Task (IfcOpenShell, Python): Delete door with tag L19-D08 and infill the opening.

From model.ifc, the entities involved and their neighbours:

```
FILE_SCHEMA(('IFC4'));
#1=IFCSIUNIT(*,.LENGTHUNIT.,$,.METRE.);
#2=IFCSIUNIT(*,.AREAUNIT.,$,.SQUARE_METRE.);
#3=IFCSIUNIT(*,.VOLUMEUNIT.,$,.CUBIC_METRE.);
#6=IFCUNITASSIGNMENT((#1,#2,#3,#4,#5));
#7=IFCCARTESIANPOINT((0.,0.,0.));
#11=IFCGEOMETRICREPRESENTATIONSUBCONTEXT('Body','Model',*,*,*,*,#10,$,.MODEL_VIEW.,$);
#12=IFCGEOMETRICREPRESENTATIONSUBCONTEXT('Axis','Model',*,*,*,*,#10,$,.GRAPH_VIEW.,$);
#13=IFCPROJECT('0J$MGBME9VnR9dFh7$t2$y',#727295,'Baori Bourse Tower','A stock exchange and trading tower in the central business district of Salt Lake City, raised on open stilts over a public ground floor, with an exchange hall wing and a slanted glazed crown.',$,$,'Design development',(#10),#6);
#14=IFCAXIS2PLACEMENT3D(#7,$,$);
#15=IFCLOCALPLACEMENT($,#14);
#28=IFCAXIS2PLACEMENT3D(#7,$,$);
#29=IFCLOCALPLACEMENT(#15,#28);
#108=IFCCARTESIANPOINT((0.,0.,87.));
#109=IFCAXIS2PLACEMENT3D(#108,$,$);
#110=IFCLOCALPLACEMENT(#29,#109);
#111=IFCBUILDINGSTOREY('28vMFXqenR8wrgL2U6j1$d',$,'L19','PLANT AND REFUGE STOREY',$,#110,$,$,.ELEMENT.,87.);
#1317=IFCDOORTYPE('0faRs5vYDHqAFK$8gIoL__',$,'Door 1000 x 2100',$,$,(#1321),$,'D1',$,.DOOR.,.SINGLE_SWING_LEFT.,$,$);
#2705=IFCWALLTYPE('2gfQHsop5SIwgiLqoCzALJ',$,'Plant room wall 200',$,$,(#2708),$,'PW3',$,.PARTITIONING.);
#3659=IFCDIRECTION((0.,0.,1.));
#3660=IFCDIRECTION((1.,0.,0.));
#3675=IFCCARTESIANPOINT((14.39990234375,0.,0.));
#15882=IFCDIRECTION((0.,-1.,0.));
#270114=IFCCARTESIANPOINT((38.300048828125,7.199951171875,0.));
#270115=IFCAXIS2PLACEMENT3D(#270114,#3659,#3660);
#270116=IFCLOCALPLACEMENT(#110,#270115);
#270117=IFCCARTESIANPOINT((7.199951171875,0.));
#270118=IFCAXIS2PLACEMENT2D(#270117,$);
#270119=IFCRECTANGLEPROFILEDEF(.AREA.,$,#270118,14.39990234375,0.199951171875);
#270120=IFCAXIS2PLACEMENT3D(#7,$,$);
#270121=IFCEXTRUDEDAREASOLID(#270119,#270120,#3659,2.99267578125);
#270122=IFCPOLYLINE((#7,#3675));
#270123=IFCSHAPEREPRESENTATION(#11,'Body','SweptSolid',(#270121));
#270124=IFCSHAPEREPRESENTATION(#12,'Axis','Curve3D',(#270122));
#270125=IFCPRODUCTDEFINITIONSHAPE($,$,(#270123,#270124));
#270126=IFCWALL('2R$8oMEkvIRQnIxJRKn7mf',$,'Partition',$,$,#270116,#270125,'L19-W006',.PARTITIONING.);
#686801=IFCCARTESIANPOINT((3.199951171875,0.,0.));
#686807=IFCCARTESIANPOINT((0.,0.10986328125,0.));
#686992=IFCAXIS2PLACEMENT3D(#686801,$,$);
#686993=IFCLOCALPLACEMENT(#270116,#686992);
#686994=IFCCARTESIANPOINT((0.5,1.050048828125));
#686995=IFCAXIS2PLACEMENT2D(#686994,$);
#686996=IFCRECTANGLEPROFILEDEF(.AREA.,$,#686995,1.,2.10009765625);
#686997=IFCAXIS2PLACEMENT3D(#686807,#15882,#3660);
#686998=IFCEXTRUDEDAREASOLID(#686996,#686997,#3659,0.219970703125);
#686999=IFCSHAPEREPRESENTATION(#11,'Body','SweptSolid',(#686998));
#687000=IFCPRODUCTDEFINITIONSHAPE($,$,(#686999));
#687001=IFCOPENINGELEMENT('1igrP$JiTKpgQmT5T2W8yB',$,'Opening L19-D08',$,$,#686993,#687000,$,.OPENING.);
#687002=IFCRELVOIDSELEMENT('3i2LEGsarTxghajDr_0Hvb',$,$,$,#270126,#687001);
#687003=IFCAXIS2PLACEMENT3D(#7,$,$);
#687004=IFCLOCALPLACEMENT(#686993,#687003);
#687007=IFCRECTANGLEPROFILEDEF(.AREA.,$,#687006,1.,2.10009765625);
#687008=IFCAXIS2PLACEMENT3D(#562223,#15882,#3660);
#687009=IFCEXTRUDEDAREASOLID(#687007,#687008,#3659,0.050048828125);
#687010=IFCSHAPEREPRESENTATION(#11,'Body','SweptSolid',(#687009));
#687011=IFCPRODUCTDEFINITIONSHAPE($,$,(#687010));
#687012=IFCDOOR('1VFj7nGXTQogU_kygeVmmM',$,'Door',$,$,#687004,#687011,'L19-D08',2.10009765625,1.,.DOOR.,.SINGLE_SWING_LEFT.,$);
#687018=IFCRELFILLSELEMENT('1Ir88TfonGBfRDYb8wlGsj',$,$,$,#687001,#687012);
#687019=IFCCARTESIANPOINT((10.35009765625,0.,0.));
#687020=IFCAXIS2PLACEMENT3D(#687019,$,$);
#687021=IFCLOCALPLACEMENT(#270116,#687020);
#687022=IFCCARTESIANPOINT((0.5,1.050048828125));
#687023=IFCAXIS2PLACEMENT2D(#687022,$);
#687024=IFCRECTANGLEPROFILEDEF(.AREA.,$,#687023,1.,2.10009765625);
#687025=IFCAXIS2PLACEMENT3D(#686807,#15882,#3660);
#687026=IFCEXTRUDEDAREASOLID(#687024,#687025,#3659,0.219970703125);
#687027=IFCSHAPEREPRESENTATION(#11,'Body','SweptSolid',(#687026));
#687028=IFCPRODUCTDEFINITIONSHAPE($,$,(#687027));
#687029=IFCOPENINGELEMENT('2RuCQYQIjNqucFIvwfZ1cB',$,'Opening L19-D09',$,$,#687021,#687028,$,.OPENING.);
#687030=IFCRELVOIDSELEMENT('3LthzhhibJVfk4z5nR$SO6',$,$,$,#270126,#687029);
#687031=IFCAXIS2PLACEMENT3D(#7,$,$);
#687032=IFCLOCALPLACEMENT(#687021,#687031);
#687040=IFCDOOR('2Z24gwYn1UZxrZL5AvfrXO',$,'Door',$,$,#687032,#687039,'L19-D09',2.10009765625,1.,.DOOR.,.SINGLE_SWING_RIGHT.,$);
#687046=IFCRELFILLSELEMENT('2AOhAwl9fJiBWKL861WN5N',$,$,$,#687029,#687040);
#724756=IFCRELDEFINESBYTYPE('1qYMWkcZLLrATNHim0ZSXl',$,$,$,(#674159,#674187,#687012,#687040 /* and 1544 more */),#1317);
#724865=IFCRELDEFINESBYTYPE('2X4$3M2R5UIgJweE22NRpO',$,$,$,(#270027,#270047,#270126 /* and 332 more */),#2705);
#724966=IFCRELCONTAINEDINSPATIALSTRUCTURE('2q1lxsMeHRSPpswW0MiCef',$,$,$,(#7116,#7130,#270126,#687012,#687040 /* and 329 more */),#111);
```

```python
import ifcopenshell
import ifcopenshell.api.feature
import ifcopenshell.api.root
import ifcopenshell.geom
import ifcopenshell.util.shape

model = ifcopenshell.open("model.ifc")
settings = ifcopenshell.geom.settings()


def volume(element):
    """Net volume in cubic metres, openings subtracted."""
    shape = ifcopenshell.geom.create_shape(settings, element)
    return ifcopenshell.util.shape.get_volume(shape.geometry)


door = model.by_id(687012)
opening = door.FillsVoids[0].RelatingOpeningElement
wall = opening.VoidsElements[0].RelatingBuildingElement
before = volume(wall)

ifcopenshell.api.root.remove_product(model, product=door)
ifcopenshell.api.feature.remove_feature(model, feature=opening)

after = volume(wall)

print(f"wall volume {before:.3f} -> {after:.3f} m3")

model.write("model_v2.ifc")
```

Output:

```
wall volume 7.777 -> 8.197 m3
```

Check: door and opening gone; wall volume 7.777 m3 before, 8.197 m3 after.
